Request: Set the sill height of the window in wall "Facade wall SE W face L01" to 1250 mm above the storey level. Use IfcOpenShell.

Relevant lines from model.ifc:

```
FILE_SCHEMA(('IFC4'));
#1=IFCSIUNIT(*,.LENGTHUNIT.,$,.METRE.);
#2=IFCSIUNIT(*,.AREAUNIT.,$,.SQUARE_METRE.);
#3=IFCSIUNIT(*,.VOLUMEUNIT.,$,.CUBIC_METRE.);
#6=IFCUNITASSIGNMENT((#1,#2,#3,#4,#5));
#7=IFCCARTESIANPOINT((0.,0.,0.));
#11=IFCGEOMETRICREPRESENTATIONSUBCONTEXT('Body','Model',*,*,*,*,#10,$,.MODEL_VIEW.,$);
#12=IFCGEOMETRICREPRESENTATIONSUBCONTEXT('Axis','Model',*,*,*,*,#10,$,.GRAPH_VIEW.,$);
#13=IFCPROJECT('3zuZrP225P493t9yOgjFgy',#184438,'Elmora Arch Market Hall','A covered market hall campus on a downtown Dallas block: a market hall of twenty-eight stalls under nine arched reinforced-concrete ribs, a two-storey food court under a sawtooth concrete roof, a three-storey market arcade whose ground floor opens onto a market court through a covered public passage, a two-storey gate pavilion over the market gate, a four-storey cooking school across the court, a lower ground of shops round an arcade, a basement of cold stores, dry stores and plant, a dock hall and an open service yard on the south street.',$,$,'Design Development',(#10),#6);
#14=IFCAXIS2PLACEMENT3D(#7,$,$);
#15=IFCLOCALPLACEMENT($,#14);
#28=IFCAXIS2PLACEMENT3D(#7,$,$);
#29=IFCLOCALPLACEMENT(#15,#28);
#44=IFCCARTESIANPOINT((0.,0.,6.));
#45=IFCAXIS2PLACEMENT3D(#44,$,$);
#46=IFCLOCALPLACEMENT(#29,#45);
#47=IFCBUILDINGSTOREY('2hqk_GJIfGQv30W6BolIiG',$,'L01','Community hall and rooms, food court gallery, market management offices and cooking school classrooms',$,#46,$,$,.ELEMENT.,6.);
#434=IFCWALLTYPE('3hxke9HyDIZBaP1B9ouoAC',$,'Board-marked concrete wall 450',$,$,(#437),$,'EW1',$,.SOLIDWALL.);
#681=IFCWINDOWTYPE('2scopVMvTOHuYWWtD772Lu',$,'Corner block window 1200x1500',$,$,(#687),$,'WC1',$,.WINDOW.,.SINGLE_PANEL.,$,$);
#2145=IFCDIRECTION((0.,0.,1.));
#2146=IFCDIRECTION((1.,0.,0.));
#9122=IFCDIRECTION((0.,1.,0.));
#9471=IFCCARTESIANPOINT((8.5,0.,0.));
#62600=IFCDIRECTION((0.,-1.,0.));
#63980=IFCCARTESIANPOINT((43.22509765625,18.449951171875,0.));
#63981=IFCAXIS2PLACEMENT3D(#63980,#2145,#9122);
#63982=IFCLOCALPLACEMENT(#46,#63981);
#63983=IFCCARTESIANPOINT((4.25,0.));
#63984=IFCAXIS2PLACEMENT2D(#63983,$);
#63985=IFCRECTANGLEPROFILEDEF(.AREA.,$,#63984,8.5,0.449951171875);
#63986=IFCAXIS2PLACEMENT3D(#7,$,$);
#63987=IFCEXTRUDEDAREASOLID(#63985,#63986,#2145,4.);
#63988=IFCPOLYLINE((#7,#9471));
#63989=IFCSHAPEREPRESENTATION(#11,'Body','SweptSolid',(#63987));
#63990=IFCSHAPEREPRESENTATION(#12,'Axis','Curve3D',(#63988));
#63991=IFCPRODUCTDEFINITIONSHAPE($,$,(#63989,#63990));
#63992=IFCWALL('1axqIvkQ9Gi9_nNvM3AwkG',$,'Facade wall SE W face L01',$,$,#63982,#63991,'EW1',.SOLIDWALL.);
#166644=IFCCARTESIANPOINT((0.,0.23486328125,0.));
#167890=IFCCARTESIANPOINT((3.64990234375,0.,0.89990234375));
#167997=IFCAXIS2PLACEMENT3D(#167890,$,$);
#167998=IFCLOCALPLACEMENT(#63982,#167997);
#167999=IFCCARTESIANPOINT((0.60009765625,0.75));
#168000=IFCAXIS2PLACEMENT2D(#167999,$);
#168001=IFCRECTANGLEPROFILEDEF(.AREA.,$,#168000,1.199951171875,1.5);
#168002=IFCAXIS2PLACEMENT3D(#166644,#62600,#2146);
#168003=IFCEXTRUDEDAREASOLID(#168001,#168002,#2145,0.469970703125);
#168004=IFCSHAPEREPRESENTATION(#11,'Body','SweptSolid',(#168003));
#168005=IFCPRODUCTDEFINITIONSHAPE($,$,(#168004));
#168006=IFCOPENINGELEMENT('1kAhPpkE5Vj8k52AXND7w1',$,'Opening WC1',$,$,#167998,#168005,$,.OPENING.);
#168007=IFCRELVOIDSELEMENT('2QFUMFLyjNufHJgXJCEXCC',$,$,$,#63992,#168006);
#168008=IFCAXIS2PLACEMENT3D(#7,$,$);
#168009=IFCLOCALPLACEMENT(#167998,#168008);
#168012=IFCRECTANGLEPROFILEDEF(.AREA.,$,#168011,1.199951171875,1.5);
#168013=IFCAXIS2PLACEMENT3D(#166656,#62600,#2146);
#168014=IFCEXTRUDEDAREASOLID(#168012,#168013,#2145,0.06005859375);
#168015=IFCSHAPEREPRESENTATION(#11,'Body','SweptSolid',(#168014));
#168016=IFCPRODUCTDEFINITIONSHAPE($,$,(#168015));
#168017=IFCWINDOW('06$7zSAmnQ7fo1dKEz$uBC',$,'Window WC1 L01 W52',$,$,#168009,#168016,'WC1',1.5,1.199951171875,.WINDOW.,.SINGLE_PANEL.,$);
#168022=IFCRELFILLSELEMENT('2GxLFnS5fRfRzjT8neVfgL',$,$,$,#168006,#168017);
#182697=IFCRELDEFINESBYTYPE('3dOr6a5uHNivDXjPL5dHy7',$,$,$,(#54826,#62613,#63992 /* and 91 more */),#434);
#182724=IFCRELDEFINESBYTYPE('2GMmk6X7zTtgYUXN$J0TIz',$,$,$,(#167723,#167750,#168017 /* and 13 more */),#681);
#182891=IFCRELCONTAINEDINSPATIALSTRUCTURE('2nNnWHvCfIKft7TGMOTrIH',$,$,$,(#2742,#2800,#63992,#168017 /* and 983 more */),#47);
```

```python
import numpy as np
import ifcopenshell
import ifcopenshell.api.geometry
import ifcopenshell.geom
import ifcopenshell.util.element
import ifcopenshell.util.placement
import ifcopenshell.util.shape
import ifcopenshell.util.unit

model = ifcopenshell.open("model.ifc")
unit_scale = ifcopenshell.util.unit.calculate_unit_scale(model)

window = model.by_id(168017)
opening = window.FillsVoids[0].RelatingOpeningElement
storey = ifcopenshell.util.element.get_container(window, ifc_class="IfcBuildingStorey")
level = ifcopenshell.util.placement.get_local_placement(storey.ObjectPlacement)[2, 3]

# The opening's origin need not be at the sill, so measure its lowest point.
shape = ifcopenshell.geom.create_shape(ifcopenshell.geom.settings(), opening)
bottom = ifcopenshell.util.shape.get_shape_bottom_elevation(shape, shape.geometry) / unit_scale
dz = level + 1.25 / unit_scale - bottom

shift = np.array([0.0, 0.0, dz])
# The window is placed relative to its opening, so it follows when the opening moves.
matrix = ifcopenshell.util.placement.get_local_placement(opening.ObjectPlacement)
matrix[:3, 3] += shift
ifcopenshell.api.geometry.edit_object_placement(
    model, product=opening, matrix=matrix, is_si=False, should_transform_children=True
)

print(f"moved by {dz * unit_scale:+.3f} m")

model.write("model-out.ifc")
```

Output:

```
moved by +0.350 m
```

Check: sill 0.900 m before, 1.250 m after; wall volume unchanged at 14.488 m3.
